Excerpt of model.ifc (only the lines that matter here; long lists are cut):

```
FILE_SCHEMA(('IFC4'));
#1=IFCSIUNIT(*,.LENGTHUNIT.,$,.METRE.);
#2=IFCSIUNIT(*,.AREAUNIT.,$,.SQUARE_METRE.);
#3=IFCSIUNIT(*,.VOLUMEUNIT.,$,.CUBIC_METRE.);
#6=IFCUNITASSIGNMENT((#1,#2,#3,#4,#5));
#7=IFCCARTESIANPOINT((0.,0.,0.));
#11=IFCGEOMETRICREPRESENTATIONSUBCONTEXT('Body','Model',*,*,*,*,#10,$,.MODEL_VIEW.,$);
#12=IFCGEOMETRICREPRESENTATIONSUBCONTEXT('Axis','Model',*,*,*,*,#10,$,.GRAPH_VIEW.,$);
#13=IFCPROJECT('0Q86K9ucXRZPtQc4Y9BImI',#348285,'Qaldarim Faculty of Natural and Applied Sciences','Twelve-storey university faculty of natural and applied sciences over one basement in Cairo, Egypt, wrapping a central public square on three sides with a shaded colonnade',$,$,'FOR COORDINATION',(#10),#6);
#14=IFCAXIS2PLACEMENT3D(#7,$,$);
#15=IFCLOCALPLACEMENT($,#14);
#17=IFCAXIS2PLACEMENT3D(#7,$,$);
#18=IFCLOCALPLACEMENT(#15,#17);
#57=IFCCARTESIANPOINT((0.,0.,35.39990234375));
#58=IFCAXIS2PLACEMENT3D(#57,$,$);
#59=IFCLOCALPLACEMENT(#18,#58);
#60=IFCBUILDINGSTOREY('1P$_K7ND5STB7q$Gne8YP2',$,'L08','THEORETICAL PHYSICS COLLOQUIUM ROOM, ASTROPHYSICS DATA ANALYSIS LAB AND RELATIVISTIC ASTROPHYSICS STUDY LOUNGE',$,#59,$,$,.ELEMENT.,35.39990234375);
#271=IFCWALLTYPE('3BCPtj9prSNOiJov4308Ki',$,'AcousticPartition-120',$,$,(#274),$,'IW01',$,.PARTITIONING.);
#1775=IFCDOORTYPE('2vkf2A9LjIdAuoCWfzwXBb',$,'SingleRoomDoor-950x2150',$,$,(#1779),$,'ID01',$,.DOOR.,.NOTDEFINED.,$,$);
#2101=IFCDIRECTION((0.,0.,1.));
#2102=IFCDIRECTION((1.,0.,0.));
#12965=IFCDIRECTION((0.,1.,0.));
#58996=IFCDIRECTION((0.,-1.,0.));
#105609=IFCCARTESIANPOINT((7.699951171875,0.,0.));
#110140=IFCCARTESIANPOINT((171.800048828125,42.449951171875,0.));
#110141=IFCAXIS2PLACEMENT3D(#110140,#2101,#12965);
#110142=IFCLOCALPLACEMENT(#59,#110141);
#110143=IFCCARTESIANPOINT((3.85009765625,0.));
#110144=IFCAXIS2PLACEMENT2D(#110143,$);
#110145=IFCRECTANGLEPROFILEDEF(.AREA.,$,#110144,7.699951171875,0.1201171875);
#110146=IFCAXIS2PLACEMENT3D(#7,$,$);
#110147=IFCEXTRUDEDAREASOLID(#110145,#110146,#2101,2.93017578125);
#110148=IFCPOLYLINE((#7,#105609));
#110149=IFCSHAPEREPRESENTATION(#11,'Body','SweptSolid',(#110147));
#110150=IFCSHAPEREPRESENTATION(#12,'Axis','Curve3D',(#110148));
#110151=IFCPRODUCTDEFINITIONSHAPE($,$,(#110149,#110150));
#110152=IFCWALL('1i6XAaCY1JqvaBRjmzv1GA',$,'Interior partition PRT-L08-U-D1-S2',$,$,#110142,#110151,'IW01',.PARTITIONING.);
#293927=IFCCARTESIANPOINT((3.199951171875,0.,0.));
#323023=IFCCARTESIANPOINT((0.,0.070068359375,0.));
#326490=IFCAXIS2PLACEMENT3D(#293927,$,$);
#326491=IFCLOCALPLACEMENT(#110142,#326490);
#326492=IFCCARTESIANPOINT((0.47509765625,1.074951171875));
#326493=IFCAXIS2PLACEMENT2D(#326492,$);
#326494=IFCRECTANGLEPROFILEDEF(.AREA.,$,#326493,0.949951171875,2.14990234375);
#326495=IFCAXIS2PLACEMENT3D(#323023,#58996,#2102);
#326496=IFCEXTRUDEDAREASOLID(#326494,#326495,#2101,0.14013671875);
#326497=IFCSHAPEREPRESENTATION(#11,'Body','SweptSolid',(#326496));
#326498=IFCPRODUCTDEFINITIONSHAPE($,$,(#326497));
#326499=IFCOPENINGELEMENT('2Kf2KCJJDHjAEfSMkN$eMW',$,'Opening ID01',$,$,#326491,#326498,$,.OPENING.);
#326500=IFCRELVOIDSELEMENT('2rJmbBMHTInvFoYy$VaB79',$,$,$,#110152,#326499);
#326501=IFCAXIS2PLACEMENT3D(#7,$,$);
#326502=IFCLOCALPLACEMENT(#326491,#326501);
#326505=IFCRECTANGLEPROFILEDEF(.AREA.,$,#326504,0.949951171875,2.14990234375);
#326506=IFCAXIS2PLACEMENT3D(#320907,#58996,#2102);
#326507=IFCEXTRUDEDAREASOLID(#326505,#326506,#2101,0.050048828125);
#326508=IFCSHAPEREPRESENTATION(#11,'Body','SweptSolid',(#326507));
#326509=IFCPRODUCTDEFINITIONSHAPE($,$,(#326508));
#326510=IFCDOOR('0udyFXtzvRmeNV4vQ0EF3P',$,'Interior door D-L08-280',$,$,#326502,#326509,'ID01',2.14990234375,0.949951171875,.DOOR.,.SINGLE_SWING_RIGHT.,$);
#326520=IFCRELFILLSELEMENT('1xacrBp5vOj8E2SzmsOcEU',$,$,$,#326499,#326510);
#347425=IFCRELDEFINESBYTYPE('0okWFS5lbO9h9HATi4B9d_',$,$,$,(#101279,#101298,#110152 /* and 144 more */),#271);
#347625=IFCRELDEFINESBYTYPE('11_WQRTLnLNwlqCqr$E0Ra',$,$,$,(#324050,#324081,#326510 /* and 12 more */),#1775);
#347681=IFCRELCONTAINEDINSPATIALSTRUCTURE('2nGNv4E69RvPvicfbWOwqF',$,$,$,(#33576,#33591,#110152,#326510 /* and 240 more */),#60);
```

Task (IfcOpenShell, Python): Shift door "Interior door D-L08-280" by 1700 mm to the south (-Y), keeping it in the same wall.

```python
import ifcopenshell
import ifcopenshell.api.geometry
import ifcopenshell.util.placement
import ifcopenshell.util.unit

model = ifcopenshell.open("model.ifc")
unit_scale = ifcopenshell.util.unit.calculate_unit_scale(model)

door = model.by_guid("0udyFXtzvRmeNV4vQ0EF3P")
opening = door.FillsVoids[0].RelatingOpeningElement
wall = opening.VoidsElements[0].RelatingBuildingElement

wall_matrix = ifcopenshell.util.placement.get_local_placement(wall.ObjectPlacement)
shift = wall_matrix[:3, 0] * -1.7 / unit_scale
before = ifcopenshell.util.placement.get_local_placement(door.ObjectPlacement)[:3, 3].copy()

# The door is placed relative to its opening, so it follows when the opening moves.
matrix = ifcopenshell.util.placement.get_local_placement(opening.ObjectPlacement)
matrix[:3, 3] += shift
ifcopenshell.api.geometry.edit_object_placement(
    model, product=opening, matrix=matrix, is_si=False, should_transform_children=True
)

after = ifcopenshell.util.placement.get_local_placement(door.ObjectPlacement)[:3, 3]
print("door moved by", (after - before).round(3) + 0.0)

model.write("model_rev.ifc")
```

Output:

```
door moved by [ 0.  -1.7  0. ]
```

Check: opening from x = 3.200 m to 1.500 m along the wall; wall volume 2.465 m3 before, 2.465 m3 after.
